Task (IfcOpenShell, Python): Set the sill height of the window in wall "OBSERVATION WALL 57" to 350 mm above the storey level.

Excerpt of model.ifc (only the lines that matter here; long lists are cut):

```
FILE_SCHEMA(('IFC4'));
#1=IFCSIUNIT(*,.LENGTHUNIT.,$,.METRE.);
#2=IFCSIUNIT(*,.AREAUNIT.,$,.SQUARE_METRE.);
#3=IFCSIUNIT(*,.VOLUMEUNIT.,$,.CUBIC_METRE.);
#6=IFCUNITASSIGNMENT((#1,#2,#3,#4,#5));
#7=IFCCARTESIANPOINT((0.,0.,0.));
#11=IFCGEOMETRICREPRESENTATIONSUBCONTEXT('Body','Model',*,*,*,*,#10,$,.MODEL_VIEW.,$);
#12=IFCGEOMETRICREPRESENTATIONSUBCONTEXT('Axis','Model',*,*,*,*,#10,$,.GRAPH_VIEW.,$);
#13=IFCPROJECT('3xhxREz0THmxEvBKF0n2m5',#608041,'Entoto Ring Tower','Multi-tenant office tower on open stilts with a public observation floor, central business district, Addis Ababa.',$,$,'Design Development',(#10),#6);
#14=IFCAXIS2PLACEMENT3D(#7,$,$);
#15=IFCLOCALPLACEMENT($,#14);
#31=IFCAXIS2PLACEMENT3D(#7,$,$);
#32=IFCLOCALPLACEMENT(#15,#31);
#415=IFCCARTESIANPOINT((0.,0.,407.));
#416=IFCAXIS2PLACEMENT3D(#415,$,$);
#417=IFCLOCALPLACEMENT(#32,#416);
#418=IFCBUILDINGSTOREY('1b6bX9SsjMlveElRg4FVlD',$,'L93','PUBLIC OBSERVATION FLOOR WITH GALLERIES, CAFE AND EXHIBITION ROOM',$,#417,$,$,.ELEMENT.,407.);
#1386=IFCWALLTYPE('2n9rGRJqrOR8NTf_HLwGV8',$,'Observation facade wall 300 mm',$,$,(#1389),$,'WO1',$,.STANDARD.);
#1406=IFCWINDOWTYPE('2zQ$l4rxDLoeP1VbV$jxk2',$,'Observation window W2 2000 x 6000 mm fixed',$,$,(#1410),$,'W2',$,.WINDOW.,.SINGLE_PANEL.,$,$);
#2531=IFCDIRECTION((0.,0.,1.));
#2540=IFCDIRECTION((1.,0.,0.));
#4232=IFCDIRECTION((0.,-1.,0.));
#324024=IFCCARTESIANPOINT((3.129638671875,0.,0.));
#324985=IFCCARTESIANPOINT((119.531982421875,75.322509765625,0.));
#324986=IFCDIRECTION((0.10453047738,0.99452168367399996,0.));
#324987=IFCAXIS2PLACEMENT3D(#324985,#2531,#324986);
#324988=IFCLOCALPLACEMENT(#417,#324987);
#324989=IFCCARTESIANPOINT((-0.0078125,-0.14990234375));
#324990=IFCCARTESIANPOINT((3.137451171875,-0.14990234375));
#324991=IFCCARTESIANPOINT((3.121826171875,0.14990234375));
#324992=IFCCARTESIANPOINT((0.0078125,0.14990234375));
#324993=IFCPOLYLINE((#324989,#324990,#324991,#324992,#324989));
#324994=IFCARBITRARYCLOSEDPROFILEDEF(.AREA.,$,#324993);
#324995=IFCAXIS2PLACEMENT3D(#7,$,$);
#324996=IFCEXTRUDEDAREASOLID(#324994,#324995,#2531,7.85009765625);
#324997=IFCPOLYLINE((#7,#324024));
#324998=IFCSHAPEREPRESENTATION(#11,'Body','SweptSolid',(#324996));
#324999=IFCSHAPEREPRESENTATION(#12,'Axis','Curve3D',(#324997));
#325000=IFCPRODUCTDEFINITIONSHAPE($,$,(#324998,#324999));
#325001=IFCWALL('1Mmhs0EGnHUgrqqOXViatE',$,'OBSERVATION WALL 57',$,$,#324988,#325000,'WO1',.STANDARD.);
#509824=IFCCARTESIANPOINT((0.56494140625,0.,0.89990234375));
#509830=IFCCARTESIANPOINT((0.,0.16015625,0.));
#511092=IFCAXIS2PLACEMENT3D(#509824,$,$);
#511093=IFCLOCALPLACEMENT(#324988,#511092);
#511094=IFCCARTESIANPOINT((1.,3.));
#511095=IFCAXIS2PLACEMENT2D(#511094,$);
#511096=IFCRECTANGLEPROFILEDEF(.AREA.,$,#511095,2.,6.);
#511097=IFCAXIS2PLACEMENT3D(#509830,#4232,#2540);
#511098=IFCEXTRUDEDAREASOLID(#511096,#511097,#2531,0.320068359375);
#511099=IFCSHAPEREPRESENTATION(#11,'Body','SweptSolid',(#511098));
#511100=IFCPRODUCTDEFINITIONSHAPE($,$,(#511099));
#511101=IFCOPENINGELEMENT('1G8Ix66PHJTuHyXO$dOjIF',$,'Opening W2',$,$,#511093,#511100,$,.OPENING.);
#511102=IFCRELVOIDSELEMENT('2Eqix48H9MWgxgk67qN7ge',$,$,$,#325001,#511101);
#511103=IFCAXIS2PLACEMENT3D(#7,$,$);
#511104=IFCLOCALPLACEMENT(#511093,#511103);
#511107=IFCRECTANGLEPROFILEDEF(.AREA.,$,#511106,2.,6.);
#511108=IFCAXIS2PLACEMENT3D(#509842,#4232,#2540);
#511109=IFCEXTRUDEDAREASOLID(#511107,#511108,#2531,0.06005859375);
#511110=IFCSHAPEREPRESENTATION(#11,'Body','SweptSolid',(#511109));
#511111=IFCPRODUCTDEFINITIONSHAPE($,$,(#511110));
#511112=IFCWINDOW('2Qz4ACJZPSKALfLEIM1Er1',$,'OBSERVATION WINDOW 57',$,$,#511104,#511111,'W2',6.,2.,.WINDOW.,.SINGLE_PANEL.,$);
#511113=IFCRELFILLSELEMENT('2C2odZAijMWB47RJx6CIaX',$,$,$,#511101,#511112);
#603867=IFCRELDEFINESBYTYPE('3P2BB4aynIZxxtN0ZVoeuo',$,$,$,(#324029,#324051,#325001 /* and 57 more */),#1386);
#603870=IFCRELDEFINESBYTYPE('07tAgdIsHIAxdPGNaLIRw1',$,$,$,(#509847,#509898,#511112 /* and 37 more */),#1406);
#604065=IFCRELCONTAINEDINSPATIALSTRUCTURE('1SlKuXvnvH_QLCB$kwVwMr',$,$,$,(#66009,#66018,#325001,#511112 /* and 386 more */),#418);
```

```python
import numpy as np
import ifcopenshell
import ifcopenshell.api.geometry
import ifcopenshell.geom
import ifcopenshell.util.element
import ifcopenshell.util.placement
import ifcopenshell.util.shape
import ifcopenshell.util.unit

model = ifcopenshell.open("model.ifc")
unit_scale = ifcopenshell.util.unit.calculate_unit_scale(model)

window = model.by_guid("2Qz4ACJZPSKALfLEIM1Er1")
opening = window.FillsVoids[0].RelatingOpeningElement
storey = ifcopenshell.util.element.get_container(window, ifc_class="IfcBuildingStorey")
level = ifcopenshell.util.placement.get_local_placement(storey.ObjectPlacement)[2, 3]

# The opening's origin need not be at the sill, so measure its lowest point.
shape = ifcopenshell.geom.create_shape(ifcopenshell.geom.settings(), opening)
bottom = ifcopenshell.util.shape.get_shape_bottom_elevation(shape, shape.geometry) / unit_scale
dz = level + 0.35 / unit_scale - bottom

shift = np.array([0.0, 0.0, dz])
# The window is placed relative to its opening, so it follows when the opening moves.
matrix = ifcopenshell.util.placement.get_local_placement(opening.ObjectPlacement)
matrix[:3, 3] += shift
ifcopenshell.api.geometry.edit_object_placement(
    model, product=opening, matrix=matrix, is_si=False, should_transform_children=True
)

print(f"moved by {dz * unit_scale:+.3f} m")

model.write("model-out.ifc")
```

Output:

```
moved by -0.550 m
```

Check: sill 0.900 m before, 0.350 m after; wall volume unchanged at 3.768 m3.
